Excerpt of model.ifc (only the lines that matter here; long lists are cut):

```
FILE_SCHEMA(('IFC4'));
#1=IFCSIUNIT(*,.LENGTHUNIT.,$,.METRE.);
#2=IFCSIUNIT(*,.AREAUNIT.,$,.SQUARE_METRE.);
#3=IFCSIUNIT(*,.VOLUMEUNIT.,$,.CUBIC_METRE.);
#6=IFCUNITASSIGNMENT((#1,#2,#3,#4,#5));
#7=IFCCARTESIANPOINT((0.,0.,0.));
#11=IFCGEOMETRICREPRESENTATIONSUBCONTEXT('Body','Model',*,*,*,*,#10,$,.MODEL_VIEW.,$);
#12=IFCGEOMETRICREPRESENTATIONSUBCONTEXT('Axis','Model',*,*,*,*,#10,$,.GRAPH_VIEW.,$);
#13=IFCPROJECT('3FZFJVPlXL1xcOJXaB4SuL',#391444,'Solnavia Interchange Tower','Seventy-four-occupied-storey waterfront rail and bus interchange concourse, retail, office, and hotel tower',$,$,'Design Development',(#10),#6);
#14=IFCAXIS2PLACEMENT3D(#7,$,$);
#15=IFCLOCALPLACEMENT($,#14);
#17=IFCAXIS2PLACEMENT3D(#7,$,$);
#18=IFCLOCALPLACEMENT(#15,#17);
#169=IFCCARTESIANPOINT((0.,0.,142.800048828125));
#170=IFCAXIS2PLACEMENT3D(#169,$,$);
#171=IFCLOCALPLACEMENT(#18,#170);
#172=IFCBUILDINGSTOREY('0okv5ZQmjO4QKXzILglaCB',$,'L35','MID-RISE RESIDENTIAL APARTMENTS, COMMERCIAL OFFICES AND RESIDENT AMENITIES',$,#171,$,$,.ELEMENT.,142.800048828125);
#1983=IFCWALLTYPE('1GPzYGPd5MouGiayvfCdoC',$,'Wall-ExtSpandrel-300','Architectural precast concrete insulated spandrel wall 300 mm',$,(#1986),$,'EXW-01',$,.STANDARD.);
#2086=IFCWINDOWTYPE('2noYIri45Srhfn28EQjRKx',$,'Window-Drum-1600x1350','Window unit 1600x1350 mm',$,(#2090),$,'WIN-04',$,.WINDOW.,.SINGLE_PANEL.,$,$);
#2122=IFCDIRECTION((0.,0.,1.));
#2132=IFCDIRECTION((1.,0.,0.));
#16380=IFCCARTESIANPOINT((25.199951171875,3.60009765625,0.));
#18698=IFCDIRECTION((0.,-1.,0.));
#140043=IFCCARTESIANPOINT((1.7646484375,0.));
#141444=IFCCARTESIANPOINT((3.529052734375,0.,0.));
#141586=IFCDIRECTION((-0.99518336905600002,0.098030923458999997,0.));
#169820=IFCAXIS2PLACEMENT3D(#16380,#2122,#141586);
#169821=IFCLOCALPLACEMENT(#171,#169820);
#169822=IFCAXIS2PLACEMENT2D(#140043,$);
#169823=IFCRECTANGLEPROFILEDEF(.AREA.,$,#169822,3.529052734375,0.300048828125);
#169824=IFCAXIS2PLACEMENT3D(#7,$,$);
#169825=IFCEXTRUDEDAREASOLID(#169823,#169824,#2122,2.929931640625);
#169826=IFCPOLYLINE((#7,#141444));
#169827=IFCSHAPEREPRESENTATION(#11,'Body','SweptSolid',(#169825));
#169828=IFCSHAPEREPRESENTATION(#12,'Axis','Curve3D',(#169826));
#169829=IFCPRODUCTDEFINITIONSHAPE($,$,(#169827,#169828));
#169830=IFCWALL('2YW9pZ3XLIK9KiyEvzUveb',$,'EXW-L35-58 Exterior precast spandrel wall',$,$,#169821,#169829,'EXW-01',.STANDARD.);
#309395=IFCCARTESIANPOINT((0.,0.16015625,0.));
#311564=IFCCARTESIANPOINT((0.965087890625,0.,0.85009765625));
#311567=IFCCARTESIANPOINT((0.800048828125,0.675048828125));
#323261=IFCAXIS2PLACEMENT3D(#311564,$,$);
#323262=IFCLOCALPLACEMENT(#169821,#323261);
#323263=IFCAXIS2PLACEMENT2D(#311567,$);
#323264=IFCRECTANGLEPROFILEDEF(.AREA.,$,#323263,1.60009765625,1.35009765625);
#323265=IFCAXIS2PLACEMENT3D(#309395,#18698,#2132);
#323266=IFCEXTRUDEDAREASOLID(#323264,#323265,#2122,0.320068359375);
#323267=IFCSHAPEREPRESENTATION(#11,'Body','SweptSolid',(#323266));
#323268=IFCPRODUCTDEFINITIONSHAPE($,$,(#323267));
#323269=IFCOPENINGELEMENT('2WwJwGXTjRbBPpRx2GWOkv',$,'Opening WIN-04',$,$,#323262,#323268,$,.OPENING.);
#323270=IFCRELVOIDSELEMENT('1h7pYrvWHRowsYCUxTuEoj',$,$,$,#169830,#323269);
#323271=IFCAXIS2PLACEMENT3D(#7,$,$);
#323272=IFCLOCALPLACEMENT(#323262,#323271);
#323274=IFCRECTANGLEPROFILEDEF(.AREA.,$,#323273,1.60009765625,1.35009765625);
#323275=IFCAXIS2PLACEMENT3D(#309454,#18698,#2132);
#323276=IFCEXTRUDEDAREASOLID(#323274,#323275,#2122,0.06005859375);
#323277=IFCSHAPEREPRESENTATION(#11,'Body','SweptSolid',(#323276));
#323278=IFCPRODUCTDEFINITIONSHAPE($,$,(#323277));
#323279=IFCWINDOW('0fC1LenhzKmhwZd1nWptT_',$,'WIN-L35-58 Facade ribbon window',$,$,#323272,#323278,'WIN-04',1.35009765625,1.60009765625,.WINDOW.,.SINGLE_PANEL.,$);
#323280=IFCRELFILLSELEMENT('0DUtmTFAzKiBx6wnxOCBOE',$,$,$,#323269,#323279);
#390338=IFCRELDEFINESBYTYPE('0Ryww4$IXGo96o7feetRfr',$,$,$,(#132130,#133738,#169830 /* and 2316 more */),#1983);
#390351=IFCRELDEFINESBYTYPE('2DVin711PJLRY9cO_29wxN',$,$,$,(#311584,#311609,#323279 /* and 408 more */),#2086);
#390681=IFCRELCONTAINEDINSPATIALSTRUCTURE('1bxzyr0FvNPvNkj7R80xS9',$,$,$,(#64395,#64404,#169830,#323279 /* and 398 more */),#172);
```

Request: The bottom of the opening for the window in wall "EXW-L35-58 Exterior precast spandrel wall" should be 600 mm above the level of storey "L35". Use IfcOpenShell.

```python
import numpy as np
import ifcopenshell
import ifcopenshell.api.geometry
import ifcopenshell.geom
import ifcopenshell.util.element
import ifcopenshell.util.placement
import ifcopenshell.util.shape
import ifcopenshell.util.unit

model = ifcopenshell.open("model.ifc")
unit_scale = ifcopenshell.util.unit.calculate_unit_scale(model)

window = model.by_id(323279)
opening = window.FillsVoids[0].RelatingOpeningElement
storey = ifcopenshell.util.element.get_container(window, ifc_class="IfcBuildingStorey")
level = ifcopenshell.util.placement.get_local_placement(storey.ObjectPlacement)[2, 3]

# The opening's origin need not be at the sill, so measure its lowest point.
shape = ifcopenshell.geom.create_shape(ifcopenshell.geom.settings(), opening)
bottom = ifcopenshell.util.shape.get_shape_bottom_elevation(shape, shape.geometry) / unit_scale
dz = level + 0.6 / unit_scale - bottom

shift = np.array([0.0, 0.0, dz])
# The window is placed relative to its opening, so it follows when the opening moves.
matrix = ifcopenshell.util.placement.get_local_placement(opening.ObjectPlacement)
matrix[:3, 3] += shift
ifcopenshell.api.geometry.edit_object_placement(
    model, product=opening, matrix=matrix, is_si=False, should_transform_children=True
)

print(f"moved by {dz * unit_scale:+.3f} m")

model.write("model_v2.ifc")
```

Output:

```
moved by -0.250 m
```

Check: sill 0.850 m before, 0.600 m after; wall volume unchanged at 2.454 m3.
